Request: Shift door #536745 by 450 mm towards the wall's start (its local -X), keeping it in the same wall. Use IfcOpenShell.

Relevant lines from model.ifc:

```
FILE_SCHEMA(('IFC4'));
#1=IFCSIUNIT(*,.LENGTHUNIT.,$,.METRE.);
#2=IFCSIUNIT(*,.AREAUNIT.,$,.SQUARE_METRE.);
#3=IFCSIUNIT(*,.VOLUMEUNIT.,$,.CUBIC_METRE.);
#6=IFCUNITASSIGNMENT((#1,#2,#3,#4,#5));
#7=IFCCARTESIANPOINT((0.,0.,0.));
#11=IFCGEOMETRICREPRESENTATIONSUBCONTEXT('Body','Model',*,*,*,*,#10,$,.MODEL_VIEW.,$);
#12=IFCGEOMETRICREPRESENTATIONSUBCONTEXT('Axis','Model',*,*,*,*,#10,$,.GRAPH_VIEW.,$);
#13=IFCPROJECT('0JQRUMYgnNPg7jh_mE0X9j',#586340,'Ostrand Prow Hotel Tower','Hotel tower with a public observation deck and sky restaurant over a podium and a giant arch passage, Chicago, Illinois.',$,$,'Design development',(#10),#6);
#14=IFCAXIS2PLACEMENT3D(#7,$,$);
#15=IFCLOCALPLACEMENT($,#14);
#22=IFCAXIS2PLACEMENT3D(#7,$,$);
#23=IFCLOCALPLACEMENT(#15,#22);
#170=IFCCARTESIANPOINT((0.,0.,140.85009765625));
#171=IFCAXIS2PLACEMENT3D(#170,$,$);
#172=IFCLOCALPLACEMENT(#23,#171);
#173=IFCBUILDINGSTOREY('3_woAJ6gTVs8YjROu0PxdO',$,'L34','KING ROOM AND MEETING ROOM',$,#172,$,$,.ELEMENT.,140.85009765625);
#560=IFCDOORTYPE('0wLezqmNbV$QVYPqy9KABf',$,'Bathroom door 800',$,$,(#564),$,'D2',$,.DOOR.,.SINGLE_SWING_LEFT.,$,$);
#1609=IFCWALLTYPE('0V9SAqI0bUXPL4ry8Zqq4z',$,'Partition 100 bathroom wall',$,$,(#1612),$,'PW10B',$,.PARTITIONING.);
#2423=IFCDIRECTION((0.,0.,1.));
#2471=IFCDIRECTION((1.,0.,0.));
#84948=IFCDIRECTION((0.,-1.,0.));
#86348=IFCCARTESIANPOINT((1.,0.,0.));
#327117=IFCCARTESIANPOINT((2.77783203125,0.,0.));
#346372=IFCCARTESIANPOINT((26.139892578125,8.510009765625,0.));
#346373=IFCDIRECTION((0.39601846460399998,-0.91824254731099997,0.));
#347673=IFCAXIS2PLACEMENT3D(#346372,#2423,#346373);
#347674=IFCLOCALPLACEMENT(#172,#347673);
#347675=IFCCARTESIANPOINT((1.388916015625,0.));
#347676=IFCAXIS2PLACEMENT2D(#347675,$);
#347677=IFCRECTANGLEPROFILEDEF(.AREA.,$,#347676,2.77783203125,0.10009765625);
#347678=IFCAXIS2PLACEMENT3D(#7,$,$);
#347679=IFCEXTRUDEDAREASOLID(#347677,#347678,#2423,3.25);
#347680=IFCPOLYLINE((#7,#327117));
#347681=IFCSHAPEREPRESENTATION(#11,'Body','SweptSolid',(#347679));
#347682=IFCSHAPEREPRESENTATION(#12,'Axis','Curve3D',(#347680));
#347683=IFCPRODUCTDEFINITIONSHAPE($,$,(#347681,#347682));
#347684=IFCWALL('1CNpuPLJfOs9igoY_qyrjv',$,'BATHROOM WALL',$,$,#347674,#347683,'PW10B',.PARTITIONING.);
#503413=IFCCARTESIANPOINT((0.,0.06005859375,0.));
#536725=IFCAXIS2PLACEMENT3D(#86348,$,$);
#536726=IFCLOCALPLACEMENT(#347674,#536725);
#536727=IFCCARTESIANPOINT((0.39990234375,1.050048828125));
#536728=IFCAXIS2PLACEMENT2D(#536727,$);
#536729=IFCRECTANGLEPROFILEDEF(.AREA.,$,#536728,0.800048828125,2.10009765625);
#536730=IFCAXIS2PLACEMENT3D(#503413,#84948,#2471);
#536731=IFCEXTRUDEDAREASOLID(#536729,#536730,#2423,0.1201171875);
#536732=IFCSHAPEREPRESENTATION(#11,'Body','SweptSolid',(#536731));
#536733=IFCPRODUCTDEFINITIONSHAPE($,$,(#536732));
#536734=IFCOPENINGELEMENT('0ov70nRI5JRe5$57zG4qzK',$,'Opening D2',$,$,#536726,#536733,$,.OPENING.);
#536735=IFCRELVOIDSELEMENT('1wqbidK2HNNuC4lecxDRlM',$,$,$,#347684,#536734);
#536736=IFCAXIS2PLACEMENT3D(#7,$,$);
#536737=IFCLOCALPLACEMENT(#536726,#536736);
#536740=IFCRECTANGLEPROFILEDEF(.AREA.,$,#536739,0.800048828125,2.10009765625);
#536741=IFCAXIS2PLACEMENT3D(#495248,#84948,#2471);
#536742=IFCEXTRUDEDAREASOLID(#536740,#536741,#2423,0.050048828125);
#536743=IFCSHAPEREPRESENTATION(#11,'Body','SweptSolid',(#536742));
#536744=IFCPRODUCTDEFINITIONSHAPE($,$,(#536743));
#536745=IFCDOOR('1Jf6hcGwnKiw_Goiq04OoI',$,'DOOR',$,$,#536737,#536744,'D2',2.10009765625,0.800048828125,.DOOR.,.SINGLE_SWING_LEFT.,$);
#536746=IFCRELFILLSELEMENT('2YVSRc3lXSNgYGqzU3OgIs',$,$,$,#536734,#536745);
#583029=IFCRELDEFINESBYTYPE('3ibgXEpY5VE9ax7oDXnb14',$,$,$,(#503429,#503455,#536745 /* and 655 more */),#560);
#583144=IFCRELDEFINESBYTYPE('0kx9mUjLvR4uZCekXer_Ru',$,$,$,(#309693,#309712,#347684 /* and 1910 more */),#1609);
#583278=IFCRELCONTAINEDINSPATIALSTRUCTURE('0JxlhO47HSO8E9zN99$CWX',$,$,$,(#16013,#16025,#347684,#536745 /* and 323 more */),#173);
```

```python
import ifcopenshell
import ifcopenshell.api.geometry
import ifcopenshell.util.placement

model = ifcopenshell.open("model.ifc")

door = model.by_guid("1Jf6hcGwnKiw_Goiq04OoI")
opening = door.FillsVoids[0].RelatingOpeningElement
wall = opening.VoidsElements[0].RelatingBuildingElement

wall_matrix = ifcopenshell.util.placement.get_local_placement(wall.ObjectPlacement)
shift = wall_matrix[:3, 0] * -0.45
before = ifcopenshell.util.placement.get_local_placement(door.ObjectPlacement)[:3, 3].copy()

# The door is placed relative to its opening, so it follows when the opening moves.
matrix = ifcopenshell.util.placement.get_local_placement(opening.ObjectPlacement)
matrix[:3, 3] += shift
ifcopenshell.api.geometry.edit_object_placement(
    model, product=opening, matrix=matrix, is_si=False, should_transform_children=True
)

after = ifcopenshell.util.placement.get_local_placement(door.ObjectPlacement)[:3, 3]
print("door moved by", (after - before).round(3) + 0.0)

model.write("model_v2.ifc")
```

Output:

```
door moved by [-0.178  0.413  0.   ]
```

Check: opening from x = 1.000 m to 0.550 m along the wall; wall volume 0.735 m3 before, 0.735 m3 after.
